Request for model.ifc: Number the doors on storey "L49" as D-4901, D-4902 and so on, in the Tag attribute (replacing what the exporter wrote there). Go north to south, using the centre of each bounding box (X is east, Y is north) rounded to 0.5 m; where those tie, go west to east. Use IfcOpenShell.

First a look at what the model holds.

```python
import ifcopenshell
import ifcopenshell.util.element
import ifcopenshell.util.placement

model = ifcopenshell.open("model.ifc")
print(model.schema)
storey = next(s for s in model.by_type("IfcBuildingStorey") if s.Name == "L49")
doors = [e for e in ifcopenshell.util.element.get_decomposition(storey) if e.is_a("IfcDoor")]
for e in sorted(doors, key=lambda e: e.id()):
    origin = ifcopenshell.util.placement.get_local_placement(e.ObjectPlacement)[:3, 3]
    print(e.id(), e.Tag, e.Name, origin.round(2) + 0.0, sep=" | ")
```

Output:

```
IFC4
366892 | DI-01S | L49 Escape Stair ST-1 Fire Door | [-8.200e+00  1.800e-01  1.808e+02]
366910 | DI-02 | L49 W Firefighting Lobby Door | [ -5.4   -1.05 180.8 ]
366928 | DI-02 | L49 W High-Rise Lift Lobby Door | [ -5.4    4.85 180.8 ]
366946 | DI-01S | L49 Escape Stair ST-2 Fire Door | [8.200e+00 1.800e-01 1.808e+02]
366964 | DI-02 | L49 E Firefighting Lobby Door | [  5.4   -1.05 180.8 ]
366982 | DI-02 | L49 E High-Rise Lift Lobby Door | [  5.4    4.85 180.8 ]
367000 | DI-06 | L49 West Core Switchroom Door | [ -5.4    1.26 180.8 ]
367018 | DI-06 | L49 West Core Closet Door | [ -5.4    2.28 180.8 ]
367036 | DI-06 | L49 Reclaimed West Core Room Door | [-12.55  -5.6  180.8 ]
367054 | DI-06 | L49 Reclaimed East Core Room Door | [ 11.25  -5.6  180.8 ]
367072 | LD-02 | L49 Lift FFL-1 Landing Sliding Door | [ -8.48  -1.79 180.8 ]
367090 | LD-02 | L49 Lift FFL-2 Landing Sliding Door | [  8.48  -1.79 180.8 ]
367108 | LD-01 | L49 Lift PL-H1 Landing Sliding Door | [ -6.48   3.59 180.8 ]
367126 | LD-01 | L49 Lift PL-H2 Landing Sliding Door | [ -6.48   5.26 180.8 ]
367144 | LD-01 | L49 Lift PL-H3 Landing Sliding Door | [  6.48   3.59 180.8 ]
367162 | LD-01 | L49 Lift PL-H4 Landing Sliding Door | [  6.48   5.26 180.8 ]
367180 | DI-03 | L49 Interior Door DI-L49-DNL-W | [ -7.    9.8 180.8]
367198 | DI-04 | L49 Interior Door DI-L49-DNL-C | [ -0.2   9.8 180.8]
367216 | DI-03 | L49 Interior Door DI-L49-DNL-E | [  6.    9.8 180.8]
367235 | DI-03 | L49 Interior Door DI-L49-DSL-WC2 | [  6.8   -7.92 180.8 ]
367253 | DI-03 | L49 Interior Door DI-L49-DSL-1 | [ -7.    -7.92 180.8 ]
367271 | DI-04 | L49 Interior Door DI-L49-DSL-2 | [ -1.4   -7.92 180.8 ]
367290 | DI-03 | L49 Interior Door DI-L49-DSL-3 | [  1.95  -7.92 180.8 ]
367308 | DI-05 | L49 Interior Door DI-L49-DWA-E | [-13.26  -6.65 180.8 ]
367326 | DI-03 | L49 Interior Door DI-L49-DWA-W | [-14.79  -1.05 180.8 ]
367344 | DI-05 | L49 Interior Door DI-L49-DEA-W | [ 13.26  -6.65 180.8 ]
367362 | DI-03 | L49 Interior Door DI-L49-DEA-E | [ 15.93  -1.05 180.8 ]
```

```python
import ifcopenshell
import ifcopenshell.geom
import ifcopenshell.util.element
import ifcopenshell.util.shape

model = ifcopenshell.open("model.ifc")
settings = ifcopenshell.geom.settings()
settings.set("use-world-coords", True)


def centre(element):
    shape = ifcopenshell.geom.create_shape(settings, element)
    return ifcopenshell.util.shape.get_bbox_centroid(shape.geometry)


storey = next(s for s in model.by_type("IfcBuildingStorey") if s.Name == "L49")
doors = [e for e in ifcopenshell.util.element.get_decomposition(storey) if e.is_a("IfcDoor")]

# Insertion points can sit at a corner or the storey origin, so sort by the geometry (in metres).
centres = {e: centre(e) for e in doors}
doors.sort(key=lambda e: (-round(centres[e][1] / 0.5), centres[e][0]))

for i, e in enumerate(doors, start=1):
    number = f"D-49{i:02d}"
    e.Tag = number
    print(e.id(), number)

model.write("model_v2.ifc")
```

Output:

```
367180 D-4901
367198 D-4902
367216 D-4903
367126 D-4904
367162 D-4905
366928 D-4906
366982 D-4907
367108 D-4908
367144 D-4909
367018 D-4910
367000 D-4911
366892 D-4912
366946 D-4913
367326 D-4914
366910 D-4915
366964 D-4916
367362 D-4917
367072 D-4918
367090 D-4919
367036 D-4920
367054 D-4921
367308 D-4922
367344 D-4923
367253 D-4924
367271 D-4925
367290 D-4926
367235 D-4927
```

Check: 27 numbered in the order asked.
